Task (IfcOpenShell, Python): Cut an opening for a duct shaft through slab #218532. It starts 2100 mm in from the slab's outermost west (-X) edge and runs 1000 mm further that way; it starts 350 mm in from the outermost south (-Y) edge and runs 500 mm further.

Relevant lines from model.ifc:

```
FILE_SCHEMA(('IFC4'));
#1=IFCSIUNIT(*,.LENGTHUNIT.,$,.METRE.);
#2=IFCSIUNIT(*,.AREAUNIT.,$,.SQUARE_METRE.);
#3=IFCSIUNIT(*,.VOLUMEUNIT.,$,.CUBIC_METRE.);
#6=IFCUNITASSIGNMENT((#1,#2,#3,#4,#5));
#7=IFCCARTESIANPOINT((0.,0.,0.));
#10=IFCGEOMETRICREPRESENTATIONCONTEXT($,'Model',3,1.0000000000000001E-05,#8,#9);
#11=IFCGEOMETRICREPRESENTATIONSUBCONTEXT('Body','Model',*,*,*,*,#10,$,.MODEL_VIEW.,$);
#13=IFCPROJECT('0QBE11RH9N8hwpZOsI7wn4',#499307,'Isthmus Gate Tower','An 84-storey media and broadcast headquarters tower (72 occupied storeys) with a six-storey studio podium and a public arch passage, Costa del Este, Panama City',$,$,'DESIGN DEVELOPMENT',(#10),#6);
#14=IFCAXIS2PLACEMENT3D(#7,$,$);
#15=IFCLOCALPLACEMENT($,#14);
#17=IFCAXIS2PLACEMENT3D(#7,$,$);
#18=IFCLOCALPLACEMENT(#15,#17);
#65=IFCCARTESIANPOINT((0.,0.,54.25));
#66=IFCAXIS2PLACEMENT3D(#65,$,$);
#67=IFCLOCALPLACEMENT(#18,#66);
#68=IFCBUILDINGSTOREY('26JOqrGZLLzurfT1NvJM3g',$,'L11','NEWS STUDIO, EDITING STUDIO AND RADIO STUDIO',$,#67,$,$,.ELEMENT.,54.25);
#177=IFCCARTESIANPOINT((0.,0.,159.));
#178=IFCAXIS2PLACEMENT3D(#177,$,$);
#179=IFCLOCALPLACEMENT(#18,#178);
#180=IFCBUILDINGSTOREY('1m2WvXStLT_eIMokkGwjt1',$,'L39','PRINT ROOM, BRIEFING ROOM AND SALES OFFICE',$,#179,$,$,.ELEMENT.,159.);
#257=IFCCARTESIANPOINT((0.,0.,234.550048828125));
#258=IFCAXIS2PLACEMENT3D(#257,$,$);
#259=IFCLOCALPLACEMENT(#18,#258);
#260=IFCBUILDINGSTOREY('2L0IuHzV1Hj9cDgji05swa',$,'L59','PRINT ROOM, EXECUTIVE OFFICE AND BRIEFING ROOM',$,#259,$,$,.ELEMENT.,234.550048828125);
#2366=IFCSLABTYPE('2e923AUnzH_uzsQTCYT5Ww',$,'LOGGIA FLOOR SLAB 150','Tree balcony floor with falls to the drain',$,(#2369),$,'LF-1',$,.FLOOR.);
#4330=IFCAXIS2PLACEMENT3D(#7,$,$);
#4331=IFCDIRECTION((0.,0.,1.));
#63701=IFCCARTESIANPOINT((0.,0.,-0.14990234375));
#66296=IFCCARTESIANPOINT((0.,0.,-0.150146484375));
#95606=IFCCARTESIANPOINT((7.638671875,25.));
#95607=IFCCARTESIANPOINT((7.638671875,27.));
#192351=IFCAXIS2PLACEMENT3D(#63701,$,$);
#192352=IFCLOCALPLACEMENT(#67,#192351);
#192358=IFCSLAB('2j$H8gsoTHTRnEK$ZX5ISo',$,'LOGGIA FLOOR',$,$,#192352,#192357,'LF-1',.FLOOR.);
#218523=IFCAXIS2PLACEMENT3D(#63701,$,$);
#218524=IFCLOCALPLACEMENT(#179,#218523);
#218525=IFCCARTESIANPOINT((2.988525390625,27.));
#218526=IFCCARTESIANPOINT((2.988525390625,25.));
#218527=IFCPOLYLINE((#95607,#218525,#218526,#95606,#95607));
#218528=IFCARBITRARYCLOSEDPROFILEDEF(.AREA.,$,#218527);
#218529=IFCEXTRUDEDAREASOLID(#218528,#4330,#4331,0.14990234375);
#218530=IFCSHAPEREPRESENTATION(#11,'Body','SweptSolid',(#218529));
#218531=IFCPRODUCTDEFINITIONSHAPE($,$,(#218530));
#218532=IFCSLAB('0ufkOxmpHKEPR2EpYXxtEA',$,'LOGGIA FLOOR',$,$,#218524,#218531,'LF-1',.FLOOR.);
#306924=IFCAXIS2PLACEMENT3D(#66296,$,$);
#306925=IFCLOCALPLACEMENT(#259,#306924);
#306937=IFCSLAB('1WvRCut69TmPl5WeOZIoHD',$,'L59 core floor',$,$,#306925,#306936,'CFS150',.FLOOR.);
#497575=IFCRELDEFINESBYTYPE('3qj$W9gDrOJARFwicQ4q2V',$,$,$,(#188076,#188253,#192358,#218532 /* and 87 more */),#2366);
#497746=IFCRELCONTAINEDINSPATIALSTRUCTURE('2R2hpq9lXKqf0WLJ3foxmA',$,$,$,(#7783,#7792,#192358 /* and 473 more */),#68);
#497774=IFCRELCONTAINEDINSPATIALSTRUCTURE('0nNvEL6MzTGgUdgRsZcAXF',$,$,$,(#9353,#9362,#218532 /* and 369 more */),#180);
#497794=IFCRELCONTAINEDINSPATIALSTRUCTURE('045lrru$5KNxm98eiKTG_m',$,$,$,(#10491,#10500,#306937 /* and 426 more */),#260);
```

```python
import numpy as np
import ifcopenshell
import ifcopenshell.api.feature
import ifcopenshell.api.geometry
import ifcopenshell.api.root
import ifcopenshell.geom
import ifcopenshell.util.placement
import ifcopenshell.util.representation
import ifcopenshell.util.shape
import ifcopenshell.util.unit

model = ifcopenshell.open("model.ifc")
unit_scale = ifcopenshell.util.unit.calculate_unit_scale(model)
settings = ifcopenshell.geom.settings()


def volume(element):
    """Net volume in cubic metres, openings subtracted."""
    shape = ifcopenshell.geom.create_shape(settings, element)
    return ifcopenshell.util.shape.get_volume(shape.geometry)


slab = model.by_guid("0ufkOxmpHKEPR2EpYXxtEA")
before = volume(slab)

# Extent in the slab's own axes, in metres. The edges named are its -X and -Y sides.
slab_shape = ifcopenshell.geom.create_shape(settings, slab)
vertices = ifcopenshell.util.shape.get_vertices(slab_shape.geometry)
x_min, y_min, bottom = vertices.min(axis=0)
top = vertices[:, 2].max()

opening = ifcopenshell.api.root.create_entity(model, ifc_class="IfcOpeningElement", name="Duct shaft opening", predefined_type="OPENING")
context = ifcopenshell.util.representation.get_context(model, "Model", "Body", "MODEL_VIEW")
width, depth = 1, 0.5
outline = [(0.0, 0.0), (width, 0.0), (width, depth), (0.0, depth), (0.0, 0.0)]
# Overshoot both faces by 50 mm so the cut is clean.
shape = ifcopenshell.api.geometry.add_slab_representation(
    model, context=context, depth=top - bottom + 0.1, polyline=outline
)
ifcopenshell.api.geometry.assign_representation(model, product=opening, representation=shape)

matrix = ifcopenshell.util.placement.get_local_placement(slab.ObjectPlacement)
matrix[:, 3] = matrix @ np.append(np.array([x_min + 2.1, y_min + 0.35, bottom - 0.05]) / unit_scale, 1.0)
ifcopenshell.api.geometry.edit_object_placement(model, product=opening, matrix=matrix, is_si=False)
ifcopenshell.api.feature.add_feature(model, feature=opening, element=slab)

after = volume(slab)

print(f"slab volume {before:.3f} -> {after:.3f} m3")

model.write("model_updated.ifc")
```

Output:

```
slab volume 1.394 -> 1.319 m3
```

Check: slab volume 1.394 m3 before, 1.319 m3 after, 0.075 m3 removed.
